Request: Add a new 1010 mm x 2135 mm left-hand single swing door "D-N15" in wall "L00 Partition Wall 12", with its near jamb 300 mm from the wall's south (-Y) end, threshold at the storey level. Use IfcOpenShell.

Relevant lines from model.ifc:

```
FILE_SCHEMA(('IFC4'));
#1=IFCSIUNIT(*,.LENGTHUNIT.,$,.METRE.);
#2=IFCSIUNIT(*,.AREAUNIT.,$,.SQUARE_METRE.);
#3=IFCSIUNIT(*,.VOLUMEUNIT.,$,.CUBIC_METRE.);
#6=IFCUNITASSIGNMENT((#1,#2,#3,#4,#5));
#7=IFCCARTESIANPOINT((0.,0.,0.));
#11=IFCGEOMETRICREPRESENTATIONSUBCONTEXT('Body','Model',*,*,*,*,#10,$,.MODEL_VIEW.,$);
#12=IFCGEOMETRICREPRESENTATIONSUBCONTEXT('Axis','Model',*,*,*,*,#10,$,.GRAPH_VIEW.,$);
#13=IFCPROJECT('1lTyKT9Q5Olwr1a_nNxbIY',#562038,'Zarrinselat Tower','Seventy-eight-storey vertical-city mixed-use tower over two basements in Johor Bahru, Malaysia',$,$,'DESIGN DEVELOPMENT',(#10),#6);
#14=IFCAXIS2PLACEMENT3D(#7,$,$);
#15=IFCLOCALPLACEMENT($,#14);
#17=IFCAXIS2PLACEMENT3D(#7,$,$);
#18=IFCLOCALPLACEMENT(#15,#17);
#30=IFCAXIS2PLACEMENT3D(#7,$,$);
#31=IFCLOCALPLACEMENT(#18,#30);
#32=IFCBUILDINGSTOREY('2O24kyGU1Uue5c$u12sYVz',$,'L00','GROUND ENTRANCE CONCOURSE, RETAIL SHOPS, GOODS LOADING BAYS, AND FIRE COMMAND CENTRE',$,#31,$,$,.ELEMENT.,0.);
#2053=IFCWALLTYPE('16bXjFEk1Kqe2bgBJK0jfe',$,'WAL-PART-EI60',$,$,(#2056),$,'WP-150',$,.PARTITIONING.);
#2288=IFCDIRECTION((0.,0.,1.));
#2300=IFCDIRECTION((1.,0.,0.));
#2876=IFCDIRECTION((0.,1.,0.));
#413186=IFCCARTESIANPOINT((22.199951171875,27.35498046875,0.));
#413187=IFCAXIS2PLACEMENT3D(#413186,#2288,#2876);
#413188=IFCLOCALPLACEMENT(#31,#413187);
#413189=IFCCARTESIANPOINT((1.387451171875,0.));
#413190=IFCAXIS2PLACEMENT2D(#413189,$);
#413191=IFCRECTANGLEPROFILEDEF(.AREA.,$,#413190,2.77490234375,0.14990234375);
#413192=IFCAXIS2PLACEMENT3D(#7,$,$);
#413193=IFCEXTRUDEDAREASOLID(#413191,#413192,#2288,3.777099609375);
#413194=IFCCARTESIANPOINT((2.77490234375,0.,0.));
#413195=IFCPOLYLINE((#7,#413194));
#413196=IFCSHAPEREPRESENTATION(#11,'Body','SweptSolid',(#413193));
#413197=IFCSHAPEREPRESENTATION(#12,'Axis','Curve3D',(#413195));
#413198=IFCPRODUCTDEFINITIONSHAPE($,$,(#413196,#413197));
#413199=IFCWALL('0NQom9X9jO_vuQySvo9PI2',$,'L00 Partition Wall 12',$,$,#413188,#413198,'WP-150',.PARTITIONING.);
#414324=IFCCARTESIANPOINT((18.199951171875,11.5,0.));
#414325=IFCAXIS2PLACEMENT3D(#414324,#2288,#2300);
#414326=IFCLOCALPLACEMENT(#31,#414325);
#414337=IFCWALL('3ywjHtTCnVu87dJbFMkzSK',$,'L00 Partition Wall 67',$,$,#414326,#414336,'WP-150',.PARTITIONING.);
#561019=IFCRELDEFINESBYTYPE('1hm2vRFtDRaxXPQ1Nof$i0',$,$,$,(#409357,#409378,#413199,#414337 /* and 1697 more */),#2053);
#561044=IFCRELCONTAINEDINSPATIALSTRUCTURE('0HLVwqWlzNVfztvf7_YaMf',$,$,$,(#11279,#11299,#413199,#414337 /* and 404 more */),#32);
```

```python
import numpy as np
import ifcopenshell
import ifcopenshell.api.feature
import ifcopenshell.api.geometry
import ifcopenshell.api.root
import ifcopenshell.api.spatial
import ifcopenshell.geom
import ifcopenshell.util.element
import ifcopenshell.util.placement
import ifcopenshell.util.representation
import ifcopenshell.util.shape
import ifcopenshell.util.unit

model = ifcopenshell.open("model.ifc")
unit_scale = ifcopenshell.util.unit.calculate_unit_scale(model)
settings = ifcopenshell.geom.settings()


def volume(element):
    """Net volume in cubic metres, openings subtracted."""
    shape = ifcopenshell.geom.create_shape(settings, element)
    return ifcopenshell.util.shape.get_volume(shape.geometry)


wall = model.by_guid("0NQom9X9jO_vuQySvo9PI2")
storey = ifcopenshell.util.element.get_container(wall, ifc_class="IfcBuildingStorey")
context = ifcopenshell.util.representation.get_context(model, "Model", "Body", "MODEL_VIEW")
before = volume(wall)

width, height, from_end, sill = 1.01, 2.135, 0.3, 0.0  # metres

# The wall runs along its own X axis, and the end named is its -X end.
wall_shape = ifcopenshell.geom.create_shape(settings, wall)
x, y, z = ifcopenshell.util.shape.get_vertices(wall_shape.geometry).T
start = x.min() + from_end
face, thickness = float(y.min()), float(y.max() - y.min())
wall_matrix = ifcopenshell.util.placement.get_local_placement(wall.ObjectPlacement)
level = ifcopenshell.util.placement.get_local_placement(storey.ObjectPlacement)[2, 3]


def in_wall(x, y):
    """Placement at x, y metres in the wall's axes, at sill height."""
    matrix = wall_matrix.copy()
    matrix[:, 3] = wall_matrix @ np.array([x / unit_scale, y / unit_scale, 0.0, 1.0])
    matrix[2, 3] = level + sill / unit_scale
    return matrix


# Opening: a box that overshoots both wall faces by 50 mm.
opening = ifcopenshell.api.root.create_entity(model, ifc_class="IfcOpeningElement", predefined_type="OPENING")
box = ifcopenshell.api.geometry.add_wall_representation(
    model, context=context, length=width, height=height, thickness=thickness + 0.1
)
ifcopenshell.api.geometry.assign_representation(model, product=opening, representation=box)
ifcopenshell.api.geometry.edit_object_placement(model, product=opening, matrix=in_wall(start, face - 0.05), is_si=False)
ifcopenshell.api.feature.add_feature(model, feature=opening, element=wall)

door = ifcopenshell.api.root.create_entity(model, ifc_class="IfcDoor", name="D-N15", predefined_type="DOOR")
door.OverallWidth, door.OverallHeight = width / unit_scale, height / unit_scale
door.OperationType = "SINGLE_SWING_LEFT"
body = ifcopenshell.api.geometry.add_door_representation(
    model,
    context=context,
    overall_width=door.OverallWidth,
    overall_height=door.OverallHeight,
    operation_type="SINGLE_SWING_LEFT",
    lining_properties={"LiningDepth": thickness / unit_scale, "ThresholdDepth": thickness / unit_scale},
)
ifcopenshell.api.geometry.assign_representation(model, product=door, representation=body)
ifcopenshell.api.spatial.assign_container(model, products=[door], relating_structure=storey)
ifcopenshell.api.feature.add_filling(model, opening=opening, element=door)

# The lining spans the wall, so the door starts at the wall face.
ifcopenshell.api.geometry.edit_object_placement(model, product=door, matrix=in_wall(start, face), is_si=False)

after = volume(wall)

print(f"wall volume {before:.3f} -> {after:.3f} m3")

model.write("model_updated.ifc")
```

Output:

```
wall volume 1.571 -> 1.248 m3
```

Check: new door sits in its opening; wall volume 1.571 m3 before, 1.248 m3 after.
